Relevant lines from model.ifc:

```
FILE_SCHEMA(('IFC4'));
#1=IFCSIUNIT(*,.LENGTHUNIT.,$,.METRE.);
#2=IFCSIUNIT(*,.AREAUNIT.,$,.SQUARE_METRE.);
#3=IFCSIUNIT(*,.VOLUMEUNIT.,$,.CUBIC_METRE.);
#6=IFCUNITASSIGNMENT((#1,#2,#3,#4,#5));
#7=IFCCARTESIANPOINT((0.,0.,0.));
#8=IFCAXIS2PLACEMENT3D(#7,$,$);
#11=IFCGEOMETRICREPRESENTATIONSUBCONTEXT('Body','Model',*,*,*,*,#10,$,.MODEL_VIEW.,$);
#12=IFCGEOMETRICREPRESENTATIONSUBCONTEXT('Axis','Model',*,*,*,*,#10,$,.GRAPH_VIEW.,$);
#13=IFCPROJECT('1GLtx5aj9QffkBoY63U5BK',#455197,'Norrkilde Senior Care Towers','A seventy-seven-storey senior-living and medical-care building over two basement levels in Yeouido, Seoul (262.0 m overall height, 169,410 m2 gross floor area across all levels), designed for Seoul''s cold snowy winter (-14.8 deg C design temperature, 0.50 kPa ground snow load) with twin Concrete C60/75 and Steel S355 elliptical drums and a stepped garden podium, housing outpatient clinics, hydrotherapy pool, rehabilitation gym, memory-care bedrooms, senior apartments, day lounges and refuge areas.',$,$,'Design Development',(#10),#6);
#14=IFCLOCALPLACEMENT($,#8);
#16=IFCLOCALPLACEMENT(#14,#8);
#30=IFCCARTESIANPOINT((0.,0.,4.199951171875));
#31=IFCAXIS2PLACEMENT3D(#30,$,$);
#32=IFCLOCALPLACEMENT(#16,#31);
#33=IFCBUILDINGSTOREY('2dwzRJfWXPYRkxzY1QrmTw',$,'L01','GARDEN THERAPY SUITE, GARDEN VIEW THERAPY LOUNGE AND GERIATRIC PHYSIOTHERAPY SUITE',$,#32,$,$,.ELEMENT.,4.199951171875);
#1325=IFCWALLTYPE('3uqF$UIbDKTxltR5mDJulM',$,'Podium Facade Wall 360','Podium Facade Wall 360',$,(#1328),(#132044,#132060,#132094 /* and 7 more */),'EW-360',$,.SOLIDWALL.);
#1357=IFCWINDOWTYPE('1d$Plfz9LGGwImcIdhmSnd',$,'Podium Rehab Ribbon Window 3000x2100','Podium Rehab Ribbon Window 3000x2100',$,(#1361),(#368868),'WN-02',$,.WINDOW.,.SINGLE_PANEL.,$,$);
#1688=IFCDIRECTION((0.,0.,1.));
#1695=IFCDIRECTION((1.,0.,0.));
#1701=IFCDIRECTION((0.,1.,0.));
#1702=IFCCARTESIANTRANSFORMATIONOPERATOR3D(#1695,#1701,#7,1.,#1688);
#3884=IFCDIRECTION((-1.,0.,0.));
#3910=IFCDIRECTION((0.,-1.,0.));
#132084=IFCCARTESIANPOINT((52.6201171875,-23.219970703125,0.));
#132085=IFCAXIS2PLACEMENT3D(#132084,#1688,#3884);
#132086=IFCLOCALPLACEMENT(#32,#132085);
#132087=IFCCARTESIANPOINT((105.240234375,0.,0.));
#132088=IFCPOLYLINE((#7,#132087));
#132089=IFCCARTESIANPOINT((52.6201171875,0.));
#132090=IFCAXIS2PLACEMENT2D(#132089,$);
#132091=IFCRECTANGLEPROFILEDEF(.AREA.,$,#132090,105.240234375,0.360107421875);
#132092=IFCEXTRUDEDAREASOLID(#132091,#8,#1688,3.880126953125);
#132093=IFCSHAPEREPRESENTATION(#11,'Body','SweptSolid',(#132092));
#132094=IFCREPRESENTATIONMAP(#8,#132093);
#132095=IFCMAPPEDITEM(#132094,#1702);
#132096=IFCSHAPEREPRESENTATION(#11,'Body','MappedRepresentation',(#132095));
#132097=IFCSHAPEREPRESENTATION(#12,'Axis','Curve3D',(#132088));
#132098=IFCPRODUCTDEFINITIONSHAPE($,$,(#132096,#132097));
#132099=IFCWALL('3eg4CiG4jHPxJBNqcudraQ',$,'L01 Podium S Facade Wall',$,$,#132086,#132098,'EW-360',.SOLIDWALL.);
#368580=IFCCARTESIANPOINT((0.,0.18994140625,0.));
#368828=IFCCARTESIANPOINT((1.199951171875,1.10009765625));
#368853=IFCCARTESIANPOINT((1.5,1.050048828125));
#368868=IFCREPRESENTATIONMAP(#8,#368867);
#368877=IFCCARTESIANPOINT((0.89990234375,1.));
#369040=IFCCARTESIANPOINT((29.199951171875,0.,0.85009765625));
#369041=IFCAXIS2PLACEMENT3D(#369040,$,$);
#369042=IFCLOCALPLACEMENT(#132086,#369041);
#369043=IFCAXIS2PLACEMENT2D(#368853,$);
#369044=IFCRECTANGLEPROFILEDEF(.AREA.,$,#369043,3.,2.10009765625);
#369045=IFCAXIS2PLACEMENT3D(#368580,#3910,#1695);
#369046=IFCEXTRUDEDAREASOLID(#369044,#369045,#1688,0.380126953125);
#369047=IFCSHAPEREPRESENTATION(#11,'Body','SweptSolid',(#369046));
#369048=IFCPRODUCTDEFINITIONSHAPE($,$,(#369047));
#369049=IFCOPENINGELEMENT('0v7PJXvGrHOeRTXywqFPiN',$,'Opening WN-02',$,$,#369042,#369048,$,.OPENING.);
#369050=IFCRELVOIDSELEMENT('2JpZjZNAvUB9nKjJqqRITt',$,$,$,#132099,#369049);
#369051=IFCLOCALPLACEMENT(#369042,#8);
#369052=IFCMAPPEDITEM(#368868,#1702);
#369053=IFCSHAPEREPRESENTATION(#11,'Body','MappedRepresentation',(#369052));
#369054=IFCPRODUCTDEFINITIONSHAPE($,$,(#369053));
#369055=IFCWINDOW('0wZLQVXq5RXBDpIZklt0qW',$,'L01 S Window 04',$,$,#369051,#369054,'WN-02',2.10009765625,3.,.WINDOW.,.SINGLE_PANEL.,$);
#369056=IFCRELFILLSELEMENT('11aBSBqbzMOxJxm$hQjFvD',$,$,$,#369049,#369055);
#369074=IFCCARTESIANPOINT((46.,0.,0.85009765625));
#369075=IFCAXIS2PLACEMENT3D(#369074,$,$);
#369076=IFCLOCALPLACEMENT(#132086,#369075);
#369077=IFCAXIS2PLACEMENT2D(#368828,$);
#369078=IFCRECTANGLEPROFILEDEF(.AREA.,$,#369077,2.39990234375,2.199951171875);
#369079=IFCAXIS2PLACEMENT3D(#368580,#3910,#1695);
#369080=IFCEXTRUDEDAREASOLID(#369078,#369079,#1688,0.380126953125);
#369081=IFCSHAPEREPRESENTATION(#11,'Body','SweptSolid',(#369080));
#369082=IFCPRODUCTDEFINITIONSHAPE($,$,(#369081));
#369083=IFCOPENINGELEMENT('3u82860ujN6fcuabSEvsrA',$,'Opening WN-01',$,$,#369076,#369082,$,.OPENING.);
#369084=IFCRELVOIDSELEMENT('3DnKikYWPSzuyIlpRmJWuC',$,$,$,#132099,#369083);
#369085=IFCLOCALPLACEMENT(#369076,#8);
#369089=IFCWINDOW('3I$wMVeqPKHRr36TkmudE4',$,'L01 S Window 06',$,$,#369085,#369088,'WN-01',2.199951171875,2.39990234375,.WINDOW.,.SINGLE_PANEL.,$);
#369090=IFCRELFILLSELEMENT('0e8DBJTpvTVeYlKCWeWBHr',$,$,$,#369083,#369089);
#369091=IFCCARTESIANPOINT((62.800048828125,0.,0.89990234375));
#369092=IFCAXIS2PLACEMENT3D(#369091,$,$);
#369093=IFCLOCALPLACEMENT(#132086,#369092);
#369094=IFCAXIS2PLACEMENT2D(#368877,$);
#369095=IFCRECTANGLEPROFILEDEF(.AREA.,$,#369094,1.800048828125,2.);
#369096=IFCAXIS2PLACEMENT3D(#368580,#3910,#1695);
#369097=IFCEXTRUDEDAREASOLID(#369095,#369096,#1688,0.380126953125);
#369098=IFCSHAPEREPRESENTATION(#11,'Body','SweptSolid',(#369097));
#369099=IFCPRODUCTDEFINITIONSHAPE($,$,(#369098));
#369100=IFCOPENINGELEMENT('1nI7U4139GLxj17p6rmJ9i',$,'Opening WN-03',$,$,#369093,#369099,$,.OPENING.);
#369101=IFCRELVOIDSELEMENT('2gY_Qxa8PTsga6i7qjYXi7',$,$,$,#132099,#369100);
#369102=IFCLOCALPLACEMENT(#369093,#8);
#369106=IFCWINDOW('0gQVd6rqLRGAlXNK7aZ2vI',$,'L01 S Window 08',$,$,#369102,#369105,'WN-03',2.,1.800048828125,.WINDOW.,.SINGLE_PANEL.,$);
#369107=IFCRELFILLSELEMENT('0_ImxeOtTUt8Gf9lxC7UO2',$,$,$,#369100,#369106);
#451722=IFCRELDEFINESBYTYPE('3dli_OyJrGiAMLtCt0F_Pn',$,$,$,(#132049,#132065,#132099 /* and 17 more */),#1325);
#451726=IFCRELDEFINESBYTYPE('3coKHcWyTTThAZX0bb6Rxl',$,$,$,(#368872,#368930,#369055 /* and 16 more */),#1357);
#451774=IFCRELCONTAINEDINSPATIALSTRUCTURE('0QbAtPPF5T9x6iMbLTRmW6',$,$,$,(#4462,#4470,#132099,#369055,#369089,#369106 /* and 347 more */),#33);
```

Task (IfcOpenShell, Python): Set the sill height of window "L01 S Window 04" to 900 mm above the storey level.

```python
import numpy as np
import ifcopenshell
import ifcopenshell.api.geometry
import ifcopenshell.geom
import ifcopenshell.util.element
import ifcopenshell.util.placement
import ifcopenshell.util.shape
import ifcopenshell.util.unit

model = ifcopenshell.open("model.ifc")
unit_scale = ifcopenshell.util.unit.calculate_unit_scale(model)

window = model.by_guid("0wZLQVXq5RXBDpIZklt0qW")
opening = window.FillsVoids[0].RelatingOpeningElement
storey = ifcopenshell.util.element.get_container(window, ifc_class="IfcBuildingStorey")
level = ifcopenshell.util.placement.get_local_placement(storey.ObjectPlacement)[2, 3]

# The opening's origin need not be at the sill, so measure its lowest point.
shape = ifcopenshell.geom.create_shape(ifcopenshell.geom.settings(), opening)
bottom = ifcopenshell.util.shape.get_shape_bottom_elevation(shape, shape.geometry) / unit_scale
dz = level + 0.9 - bottom

shift = np.array([0.0, 0.0, dz])
# The window is placed relative to its opening, so it follows when the opening moves.
matrix = ifcopenshell.util.placement.get_local_placement(opening.ObjectPlacement)
matrix[:3, 3] += shift
ifcopenshell.api.geometry.edit_object_placement(
    model, product=opening, matrix=matrix, is_si=False, should_transform_children=True
)

print(f"moved by {dz * unit_scale:+.3f} m")

model.write("model-out.ifc")
```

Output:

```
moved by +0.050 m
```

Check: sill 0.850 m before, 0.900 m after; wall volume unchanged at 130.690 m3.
